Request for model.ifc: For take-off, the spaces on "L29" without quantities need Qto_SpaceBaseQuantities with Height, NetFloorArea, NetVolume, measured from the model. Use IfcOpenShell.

First a look at what the model holds.

```python
import ifcopenshell
import ifcopenshell.util.element
import ifcopenshell.util.unit

model = ifcopenshell.open("model.ifc")
print(model.schema)
for unit_type in ("LENGTHUNIT", "AREAUNIT", "VOLUMEUNIT"):
    print(unit_type, ifcopenshell.util.unit.calculate_unit_scale(model, unit_type))
storey = next(s for s in model.by_type("IfcBuildingStorey") if s.Name == "L29")
spaces = [e for e in ifcopenshell.util.element.get_decomposition(storey) if e.is_a("IfcSpace")]
for e in sorted(spaces, key=lambda e: e.id()):
    print(e.id(), e.is_a(), e.Name, list(ifcopenshell.util.element.get_psets(e, qtos_only=True)), sep=" | ")
```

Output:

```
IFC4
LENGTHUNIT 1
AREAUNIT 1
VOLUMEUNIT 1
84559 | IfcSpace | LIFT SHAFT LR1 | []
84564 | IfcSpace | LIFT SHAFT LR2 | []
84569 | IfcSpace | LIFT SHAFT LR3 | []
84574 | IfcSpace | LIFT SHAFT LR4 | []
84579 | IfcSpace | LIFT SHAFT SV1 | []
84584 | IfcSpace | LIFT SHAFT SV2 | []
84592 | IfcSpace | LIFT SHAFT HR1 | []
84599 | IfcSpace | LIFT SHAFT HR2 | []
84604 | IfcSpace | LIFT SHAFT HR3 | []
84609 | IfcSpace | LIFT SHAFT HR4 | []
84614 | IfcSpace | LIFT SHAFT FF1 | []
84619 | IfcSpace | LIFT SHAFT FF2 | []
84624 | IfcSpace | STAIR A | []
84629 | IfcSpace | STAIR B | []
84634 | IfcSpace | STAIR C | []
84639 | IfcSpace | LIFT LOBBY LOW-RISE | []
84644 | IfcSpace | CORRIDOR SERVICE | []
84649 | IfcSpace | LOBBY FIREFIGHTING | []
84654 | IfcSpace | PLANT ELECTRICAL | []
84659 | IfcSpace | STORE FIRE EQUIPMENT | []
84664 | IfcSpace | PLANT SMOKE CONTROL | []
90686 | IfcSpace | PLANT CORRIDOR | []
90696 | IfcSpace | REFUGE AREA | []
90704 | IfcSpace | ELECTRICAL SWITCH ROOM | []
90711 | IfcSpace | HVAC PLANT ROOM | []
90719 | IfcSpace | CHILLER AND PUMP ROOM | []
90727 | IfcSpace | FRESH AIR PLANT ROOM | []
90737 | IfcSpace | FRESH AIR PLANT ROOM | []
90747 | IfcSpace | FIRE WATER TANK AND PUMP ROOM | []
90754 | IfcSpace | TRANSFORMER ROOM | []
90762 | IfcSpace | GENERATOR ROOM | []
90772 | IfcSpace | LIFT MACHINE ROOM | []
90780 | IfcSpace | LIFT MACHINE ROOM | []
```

```python
import ifcopenshell
import ifcopenshell.api.pset
import ifcopenshell.geom
import ifcopenshell.util.element
import ifcopenshell.util.shape
import ifcopenshell.util.unit

model = ifcopenshell.open("model.ifc")
unit_scale = ifcopenshell.util.unit.calculate_unit_scale(model)
area_scale = ifcopenshell.util.unit.calculate_unit_scale(model, "AREAUNIT")
volume_scale = ifcopenshell.util.unit.calculate_unit_scale(model, "VOLUMEUNIT")
settings = ifcopenshell.geom.settings()

storey = next(s for s in model.by_type("IfcBuildingStorey") if s.Name == "L29")
spaces = [e for e in ifcopenshell.util.element.get_decomposition(storey) if e.is_a("IfcSpace")]

for e in sorted(spaces, key=lambda e: e.id()):
    if ifcopenshell.util.element.get_psets(e, qtos_only=True, should_inherit=False):
        continue
    # Geometry comes back in metres, in the element's own axes.
    shape = ifcopenshell.geom.create_shape(settings, e)
    values = {
        "Height": ifcopenshell.util.shape.get_z(shape.geometry) / unit_scale,
        "NetFloorArea": ifcopenshell.util.shape.get_footprint_area(shape.geometry) / area_scale,
        "NetVolume": ifcopenshell.util.shape.get_volume(shape.geometry) / volume_scale,
    }
    qto = ifcopenshell.api.pset.add_qto(model, product=e, name="Qto_SpaceBaseQuantities")
    ifcopenshell.api.pset.edit_qto(model, qto=qto, properties=values)
    print(e.id(), {k: round(v, 3) for k, v in values.items()})

model.write("model_updated.ifc")
```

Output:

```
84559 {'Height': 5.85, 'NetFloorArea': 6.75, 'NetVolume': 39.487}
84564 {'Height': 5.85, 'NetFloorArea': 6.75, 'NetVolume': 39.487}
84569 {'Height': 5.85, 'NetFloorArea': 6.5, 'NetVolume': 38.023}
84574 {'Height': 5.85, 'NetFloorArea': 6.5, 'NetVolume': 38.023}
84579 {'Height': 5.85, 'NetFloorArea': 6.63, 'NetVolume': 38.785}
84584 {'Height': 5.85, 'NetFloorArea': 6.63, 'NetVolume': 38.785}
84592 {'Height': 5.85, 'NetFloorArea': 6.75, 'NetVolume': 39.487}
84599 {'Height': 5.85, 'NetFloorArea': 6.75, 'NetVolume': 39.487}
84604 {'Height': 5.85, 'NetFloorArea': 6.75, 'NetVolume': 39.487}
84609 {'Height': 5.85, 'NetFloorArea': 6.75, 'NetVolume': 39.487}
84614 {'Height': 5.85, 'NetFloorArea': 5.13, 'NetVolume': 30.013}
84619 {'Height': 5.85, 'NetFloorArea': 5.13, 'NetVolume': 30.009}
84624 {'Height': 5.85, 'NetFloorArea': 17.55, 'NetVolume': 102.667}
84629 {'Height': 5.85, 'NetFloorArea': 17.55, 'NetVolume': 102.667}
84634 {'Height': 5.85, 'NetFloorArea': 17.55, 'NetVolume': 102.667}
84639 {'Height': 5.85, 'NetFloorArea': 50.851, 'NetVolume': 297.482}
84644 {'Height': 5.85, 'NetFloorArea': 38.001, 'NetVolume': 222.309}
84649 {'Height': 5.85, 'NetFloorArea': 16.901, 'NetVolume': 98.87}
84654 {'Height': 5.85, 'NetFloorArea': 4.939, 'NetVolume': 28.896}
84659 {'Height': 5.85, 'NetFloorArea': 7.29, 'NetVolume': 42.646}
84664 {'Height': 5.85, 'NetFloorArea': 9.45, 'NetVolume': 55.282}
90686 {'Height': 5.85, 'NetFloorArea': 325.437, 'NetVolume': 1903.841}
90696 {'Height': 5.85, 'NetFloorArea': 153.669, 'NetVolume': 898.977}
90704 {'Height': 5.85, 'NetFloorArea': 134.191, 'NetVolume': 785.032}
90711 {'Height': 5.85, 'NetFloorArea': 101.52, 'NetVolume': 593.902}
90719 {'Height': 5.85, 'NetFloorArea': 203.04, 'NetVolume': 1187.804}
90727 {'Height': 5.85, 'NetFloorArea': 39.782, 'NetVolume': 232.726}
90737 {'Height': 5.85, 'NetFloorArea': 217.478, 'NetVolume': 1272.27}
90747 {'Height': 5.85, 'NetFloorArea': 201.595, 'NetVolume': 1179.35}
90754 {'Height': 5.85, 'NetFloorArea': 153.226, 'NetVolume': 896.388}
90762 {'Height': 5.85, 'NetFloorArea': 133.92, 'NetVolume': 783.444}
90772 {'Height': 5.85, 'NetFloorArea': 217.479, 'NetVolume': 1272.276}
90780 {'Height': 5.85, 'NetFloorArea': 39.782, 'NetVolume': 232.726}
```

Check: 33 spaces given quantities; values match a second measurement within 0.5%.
